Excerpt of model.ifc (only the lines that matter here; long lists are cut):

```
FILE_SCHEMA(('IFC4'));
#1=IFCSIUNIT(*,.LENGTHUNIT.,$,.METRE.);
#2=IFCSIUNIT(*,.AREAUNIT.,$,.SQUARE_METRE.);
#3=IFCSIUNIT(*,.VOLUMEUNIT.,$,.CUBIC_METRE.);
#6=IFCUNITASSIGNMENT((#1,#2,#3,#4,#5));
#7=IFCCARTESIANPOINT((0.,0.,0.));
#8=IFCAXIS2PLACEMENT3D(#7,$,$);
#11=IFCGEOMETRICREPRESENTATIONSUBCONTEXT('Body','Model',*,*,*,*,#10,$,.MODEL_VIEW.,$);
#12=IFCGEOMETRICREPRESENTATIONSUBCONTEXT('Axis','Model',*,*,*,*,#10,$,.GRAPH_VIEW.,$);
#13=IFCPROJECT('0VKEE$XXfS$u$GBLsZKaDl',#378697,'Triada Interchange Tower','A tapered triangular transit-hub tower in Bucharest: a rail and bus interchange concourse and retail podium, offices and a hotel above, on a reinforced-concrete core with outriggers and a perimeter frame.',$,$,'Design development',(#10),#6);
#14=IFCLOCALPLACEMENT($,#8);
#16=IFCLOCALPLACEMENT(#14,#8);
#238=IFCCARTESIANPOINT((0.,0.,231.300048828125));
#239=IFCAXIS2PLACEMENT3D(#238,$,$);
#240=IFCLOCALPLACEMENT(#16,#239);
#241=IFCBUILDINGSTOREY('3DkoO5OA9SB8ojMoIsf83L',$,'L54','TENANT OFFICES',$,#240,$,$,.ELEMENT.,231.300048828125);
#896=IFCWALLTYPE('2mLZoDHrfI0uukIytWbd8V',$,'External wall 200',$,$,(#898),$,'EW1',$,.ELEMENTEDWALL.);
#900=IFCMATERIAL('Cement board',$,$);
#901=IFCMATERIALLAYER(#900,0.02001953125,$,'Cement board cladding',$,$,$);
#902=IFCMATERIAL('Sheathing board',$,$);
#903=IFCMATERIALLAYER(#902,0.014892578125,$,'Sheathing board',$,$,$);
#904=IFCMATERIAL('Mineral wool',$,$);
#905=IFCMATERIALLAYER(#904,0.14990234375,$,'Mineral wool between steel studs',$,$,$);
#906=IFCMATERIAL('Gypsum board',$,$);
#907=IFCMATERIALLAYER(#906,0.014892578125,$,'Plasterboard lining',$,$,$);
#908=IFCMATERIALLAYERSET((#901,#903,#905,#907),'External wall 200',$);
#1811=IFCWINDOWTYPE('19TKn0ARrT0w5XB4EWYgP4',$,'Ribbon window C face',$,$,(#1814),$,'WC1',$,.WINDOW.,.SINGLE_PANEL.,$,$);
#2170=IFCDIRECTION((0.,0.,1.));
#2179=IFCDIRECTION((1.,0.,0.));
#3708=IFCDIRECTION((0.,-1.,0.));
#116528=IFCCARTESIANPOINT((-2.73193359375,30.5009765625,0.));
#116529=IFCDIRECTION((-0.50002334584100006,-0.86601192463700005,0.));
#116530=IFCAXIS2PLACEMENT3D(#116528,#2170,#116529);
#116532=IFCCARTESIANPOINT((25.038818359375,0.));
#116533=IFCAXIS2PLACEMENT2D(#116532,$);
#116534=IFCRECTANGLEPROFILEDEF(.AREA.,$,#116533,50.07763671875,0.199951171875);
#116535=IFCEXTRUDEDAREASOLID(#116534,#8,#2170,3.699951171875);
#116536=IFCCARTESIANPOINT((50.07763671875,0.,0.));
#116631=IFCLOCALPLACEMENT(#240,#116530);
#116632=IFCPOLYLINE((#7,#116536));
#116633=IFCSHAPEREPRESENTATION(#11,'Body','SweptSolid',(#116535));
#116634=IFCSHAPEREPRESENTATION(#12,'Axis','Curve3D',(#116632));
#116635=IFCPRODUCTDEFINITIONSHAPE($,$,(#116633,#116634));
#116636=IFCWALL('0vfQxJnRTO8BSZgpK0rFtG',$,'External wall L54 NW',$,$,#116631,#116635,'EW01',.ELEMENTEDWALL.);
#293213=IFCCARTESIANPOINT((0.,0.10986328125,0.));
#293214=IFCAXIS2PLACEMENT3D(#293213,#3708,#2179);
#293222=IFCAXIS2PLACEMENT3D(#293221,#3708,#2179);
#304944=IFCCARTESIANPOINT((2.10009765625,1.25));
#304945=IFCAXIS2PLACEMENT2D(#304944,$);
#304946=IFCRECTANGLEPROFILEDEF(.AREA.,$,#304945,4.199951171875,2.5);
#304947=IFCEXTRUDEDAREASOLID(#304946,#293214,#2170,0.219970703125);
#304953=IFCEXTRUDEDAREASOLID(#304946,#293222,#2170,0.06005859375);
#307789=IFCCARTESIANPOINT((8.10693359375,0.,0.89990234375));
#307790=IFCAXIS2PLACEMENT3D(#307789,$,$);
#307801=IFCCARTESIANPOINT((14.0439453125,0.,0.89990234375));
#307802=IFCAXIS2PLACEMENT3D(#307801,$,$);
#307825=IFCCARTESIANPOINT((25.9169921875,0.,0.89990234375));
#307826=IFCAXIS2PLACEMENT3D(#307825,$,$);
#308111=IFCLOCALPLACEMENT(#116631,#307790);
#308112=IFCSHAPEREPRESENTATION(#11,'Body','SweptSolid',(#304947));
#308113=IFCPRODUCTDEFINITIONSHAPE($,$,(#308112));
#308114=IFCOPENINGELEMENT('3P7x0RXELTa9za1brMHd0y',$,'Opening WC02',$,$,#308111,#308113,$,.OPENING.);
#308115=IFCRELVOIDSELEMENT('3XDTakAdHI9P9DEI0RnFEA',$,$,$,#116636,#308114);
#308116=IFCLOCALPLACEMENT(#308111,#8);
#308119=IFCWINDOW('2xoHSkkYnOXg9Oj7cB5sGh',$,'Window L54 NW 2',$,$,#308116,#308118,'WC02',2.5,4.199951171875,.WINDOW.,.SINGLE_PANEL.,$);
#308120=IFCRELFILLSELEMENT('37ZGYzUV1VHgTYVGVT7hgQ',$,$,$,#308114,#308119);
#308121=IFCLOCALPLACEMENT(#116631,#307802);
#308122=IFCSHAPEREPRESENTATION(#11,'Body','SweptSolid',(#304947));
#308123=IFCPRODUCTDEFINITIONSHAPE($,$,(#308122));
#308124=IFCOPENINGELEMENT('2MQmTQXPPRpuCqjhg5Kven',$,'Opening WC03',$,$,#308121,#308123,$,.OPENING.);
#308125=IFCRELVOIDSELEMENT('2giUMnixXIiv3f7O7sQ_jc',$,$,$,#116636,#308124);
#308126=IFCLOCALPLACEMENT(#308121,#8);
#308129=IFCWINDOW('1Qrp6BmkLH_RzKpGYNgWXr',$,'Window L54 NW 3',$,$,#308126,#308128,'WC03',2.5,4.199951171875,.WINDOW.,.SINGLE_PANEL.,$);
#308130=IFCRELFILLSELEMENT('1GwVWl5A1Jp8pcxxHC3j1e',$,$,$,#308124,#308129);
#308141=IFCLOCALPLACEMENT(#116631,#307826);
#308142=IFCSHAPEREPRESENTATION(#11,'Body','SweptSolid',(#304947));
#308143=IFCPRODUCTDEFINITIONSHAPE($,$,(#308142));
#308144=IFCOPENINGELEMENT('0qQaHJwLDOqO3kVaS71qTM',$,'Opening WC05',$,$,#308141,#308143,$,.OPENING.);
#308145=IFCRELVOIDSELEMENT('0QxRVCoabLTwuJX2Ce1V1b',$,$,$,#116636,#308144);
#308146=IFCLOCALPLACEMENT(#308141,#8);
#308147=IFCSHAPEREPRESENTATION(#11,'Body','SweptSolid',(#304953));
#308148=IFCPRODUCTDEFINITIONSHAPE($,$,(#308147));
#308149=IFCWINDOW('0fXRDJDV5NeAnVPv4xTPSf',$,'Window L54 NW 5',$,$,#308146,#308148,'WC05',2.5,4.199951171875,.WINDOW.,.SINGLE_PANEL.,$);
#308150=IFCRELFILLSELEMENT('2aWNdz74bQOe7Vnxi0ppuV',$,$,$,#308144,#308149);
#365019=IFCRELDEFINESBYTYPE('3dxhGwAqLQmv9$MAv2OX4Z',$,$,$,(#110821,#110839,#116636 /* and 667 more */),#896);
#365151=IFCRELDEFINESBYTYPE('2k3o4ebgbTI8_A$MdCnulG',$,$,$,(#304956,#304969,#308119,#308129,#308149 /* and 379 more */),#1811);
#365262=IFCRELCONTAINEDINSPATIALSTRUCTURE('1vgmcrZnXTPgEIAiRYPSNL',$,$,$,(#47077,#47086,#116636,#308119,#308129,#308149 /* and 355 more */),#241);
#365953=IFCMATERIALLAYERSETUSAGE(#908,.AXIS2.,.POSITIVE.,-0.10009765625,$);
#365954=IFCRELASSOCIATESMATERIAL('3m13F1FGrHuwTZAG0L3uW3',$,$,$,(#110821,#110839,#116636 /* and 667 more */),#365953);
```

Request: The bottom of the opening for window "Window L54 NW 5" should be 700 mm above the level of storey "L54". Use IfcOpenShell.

```python
import numpy as np
import ifcopenshell
import ifcopenshell.api.geometry
import ifcopenshell.geom
import ifcopenshell.util.element
import ifcopenshell.util.placement
import ifcopenshell.util.shape
import ifcopenshell.util.unit

model = ifcopenshell.open("model.ifc")
unit_scale = ifcopenshell.util.unit.calculate_unit_scale(model)

window = model.by_guid("0fXRDJDV5NeAnVPv4xTPSf")
opening = window.FillsVoids[0].RelatingOpeningElement
storey = ifcopenshell.util.element.get_container(window, ifc_class="IfcBuildingStorey")
level = ifcopenshell.util.placement.get_local_placement(storey.ObjectPlacement)[2, 3]

# The opening's origin need not be at the sill, so measure its lowest point.
shape = ifcopenshell.geom.create_shape(ifcopenshell.geom.settings(), opening)
bottom = ifcopenshell.util.shape.get_shape_bottom_elevation(shape, shape.geometry) / unit_scale
dz = level + 0.7 / unit_scale - bottom

shift = np.array([0.0, 0.0, dz])
# The window is placed relative to its opening, so it follows when the opening moves.
matrix = ifcopenshell.util.placement.get_local_placement(opening.ObjectPlacement)
matrix[:3, 3] += shift
ifcopenshell.api.geometry.edit_object_placement(
    model, product=opening, matrix=matrix, is_si=False, should_transform_children=True
)

print(f"moved by {dz * unit_scale:+.3f} m")

model.write("model_updated.ifc")
```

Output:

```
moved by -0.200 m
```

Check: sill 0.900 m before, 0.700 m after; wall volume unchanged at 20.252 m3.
